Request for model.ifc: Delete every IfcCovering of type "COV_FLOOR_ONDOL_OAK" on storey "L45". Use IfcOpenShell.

First a look at what the model holds.

```python
import ifcopenshell
import ifcopenshell.util.element

model = ifcopenshell.open("model.ifc")
print(model.schema)
storey = next(s for s in model.by_type("IfcBuildingStorey") if s.Name == "L45")
coverings = [e for e in ifcopenshell.util.element.get_decomposition(storey) if e.is_a("IfcCovering")]
seen = {}
for e in coverings:
    element_type = ifcopenshell.util.element.get_type(e)
    name = element_type.Name if element_type not in (None, e) else None
    seen[name] = seen.get(name, 0) + 1
for name, count in sorted(seen.items(), key=str):
    print(count, "x", name)
```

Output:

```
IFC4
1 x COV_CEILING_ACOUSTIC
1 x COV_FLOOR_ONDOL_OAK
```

```python
import ifcopenshell
import ifcopenshell.api.root
import ifcopenshell.util.element

model = ifcopenshell.open("model.ifc")

storey = next(s for s in model.by_type("IfcBuildingStorey") if s.Name == "L45")
coverings = [e for e in ifcopenshell.util.element.get_decomposition(storey) if e.is_a("IfcCovering")]
targets = [e for e in coverings if (t := ifcopenshell.util.element.get_type(e)) not in (None, e) and t.Name == "COV_FLOOR_ONDOL_OAK"]

for e in targets:
    ifcopenshell.api.root.remove_product(model, product=e)
print(len(targets), "removed")

model.write("model_updated.ifc")
```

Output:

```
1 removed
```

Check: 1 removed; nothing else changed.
